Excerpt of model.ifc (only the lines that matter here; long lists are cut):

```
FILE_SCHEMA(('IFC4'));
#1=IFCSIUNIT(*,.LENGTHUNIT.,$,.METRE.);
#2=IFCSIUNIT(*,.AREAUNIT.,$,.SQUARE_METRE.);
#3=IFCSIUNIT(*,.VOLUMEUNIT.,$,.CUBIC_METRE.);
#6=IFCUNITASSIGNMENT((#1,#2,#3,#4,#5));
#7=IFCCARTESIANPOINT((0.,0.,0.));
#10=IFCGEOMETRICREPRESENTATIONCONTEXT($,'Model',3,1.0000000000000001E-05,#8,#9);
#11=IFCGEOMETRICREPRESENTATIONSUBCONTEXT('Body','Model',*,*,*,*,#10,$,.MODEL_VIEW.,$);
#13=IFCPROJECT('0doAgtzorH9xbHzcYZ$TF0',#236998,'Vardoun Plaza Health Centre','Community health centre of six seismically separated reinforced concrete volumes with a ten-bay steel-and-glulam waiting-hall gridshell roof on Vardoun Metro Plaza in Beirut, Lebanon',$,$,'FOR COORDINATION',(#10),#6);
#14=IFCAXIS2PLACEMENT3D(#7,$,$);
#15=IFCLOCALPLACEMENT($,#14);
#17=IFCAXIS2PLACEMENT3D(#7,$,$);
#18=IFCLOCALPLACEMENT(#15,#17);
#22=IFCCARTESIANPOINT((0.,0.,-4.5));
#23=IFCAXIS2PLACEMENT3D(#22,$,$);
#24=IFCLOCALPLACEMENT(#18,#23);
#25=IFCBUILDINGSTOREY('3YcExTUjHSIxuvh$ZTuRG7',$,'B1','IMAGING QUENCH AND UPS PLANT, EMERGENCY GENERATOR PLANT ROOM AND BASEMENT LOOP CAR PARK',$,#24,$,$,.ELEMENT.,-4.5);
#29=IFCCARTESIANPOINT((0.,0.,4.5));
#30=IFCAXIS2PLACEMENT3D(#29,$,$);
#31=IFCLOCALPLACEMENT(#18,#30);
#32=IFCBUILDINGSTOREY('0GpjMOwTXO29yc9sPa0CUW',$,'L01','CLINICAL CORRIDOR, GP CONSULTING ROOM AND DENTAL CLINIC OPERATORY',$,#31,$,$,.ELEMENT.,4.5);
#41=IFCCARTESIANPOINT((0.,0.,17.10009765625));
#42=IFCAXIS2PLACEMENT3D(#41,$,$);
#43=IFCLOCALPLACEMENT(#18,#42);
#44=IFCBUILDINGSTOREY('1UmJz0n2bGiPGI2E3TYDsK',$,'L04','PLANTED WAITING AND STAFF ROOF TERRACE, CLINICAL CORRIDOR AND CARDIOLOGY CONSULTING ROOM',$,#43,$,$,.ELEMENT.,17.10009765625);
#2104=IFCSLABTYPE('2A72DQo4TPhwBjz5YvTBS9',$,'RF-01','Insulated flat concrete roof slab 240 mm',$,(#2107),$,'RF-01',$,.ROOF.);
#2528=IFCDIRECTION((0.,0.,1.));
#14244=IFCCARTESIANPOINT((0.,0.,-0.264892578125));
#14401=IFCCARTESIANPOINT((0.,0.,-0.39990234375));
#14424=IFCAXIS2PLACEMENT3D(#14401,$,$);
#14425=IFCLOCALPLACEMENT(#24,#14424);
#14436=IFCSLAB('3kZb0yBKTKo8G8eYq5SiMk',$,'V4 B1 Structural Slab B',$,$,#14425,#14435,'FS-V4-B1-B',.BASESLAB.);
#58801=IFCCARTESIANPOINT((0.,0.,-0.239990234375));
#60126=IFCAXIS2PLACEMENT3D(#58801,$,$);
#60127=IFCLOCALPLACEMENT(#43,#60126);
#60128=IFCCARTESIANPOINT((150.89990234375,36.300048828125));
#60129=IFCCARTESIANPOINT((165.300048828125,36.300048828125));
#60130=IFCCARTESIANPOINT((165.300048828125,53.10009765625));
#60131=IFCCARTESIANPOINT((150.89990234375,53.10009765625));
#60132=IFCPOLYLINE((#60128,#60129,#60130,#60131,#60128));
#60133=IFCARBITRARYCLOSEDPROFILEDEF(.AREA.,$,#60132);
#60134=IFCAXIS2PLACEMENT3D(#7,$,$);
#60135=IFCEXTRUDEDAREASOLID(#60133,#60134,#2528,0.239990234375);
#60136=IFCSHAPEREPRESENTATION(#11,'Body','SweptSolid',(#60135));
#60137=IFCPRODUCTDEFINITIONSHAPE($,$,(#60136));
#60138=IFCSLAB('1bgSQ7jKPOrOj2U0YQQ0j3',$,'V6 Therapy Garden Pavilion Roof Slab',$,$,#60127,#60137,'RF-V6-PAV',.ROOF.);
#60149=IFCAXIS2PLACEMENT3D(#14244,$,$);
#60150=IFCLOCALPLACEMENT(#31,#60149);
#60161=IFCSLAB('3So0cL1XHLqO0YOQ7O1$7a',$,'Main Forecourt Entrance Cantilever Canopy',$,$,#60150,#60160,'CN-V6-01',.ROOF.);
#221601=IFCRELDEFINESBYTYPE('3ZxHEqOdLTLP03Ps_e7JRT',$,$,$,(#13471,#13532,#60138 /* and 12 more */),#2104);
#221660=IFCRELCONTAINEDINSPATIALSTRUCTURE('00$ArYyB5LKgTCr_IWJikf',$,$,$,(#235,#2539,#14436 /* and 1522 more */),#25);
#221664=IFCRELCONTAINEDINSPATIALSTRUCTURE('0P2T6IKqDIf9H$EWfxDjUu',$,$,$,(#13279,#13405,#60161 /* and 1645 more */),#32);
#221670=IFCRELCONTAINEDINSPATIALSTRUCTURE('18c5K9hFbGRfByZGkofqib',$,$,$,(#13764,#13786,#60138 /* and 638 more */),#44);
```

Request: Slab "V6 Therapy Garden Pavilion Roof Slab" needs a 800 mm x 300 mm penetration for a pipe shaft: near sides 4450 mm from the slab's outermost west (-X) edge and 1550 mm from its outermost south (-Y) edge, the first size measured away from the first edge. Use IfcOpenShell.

```python
import numpy as np
import ifcopenshell
import ifcopenshell.api.feature
import ifcopenshell.api.geometry
import ifcopenshell.api.root
import ifcopenshell.geom
import ifcopenshell.util.placement
import ifcopenshell.util.representation
import ifcopenshell.util.shape
import ifcopenshell.util.unit

model = ifcopenshell.open("model.ifc")
unit_scale = ifcopenshell.util.unit.calculate_unit_scale(model)
settings = ifcopenshell.geom.settings()


def volume(element):
    """Net volume in cubic metres, openings subtracted."""
    shape = ifcopenshell.geom.create_shape(settings, element)
    return ifcopenshell.util.shape.get_volume(shape.geometry)


slab = model.by_id(60138)
before = volume(slab)

# Extent in the slab's own axes, in metres. The edges named are its -X and -Y sides.
slab_shape = ifcopenshell.geom.create_shape(settings, slab)
vertices = ifcopenshell.util.shape.get_vertices(slab_shape.geometry)
x_min, y_min, bottom = vertices.min(axis=0)
top = vertices[:, 2].max()

opening = ifcopenshell.api.root.create_entity(model, ifc_class="IfcOpeningElement", name="Pipe shaft opening", predefined_type="OPENING")
context = ifcopenshell.util.representation.get_context(model, "Model", "Body", "MODEL_VIEW")
width, depth = 0.8, 0.3
outline = [(0.0, 0.0), (width, 0.0), (width, depth), (0.0, depth), (0.0, 0.0)]
# Overshoot both faces by 50 mm so the cut is clean.
shape = ifcopenshell.api.geometry.add_slab_representation(
    model, context=context, depth=top - bottom + 0.1, polyline=outline
)
ifcopenshell.api.geometry.assign_representation(model, product=opening, representation=shape)

matrix = ifcopenshell.util.placement.get_local_placement(slab.ObjectPlacement)
matrix[:, 3] = matrix @ np.append(np.array([x_min + 4.45, y_min + 1.55, bottom - 0.05]) / unit_scale, 1.0)
ifcopenshell.api.geometry.edit_object_placement(model, product=opening, matrix=matrix, is_si=False)
ifcopenshell.api.feature.add_feature(model, feature=opening, element=slab)

after = volume(slab)

print(f"slab volume {before:.3f} -> {after:.3f} m3")

model.write("model_edited.ifc")
```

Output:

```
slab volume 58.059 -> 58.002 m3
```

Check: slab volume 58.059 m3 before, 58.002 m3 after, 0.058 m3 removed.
